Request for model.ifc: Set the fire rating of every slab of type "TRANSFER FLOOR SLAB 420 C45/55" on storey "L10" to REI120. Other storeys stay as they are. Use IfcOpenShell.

First a look at what the model holds.

```python
import ifcopenshell
import ifcopenshell.util.element

model = ifcopenshell.open("model.ifc")
print(model.schema)
storey = next(s for s in model.by_type("IfcBuildingStorey") if s.Name == "L10")
slabs = [e for e in ifcopenshell.util.element.get_decomposition(storey) if e.is_a("IfcSlab")]
seen = {}
for e in slabs:
    element_type = ifcopenshell.util.element.get_type(e)
    key = (element_type.Name if element_type != e and element_type else None, ifcopenshell.util.element.get_pset(e, "Pset_SlabCommon", "FireRating"))
    seen[key] = seen.get(key, 0) + 1
for (name, value), count in sorted(seen.items(), key=str):
    print(count, "x", name, "|", value)
```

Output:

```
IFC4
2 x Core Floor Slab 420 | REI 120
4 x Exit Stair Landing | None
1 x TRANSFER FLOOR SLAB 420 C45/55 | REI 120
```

```python
import ifcopenshell
import ifcopenshell.api.pset
import ifcopenshell.util.element

model = ifcopenshell.open("model.ifc")

storey = next(s for s in model.by_type("IfcBuildingStorey") if s.Name == "L10")
slabs = [e for e in ifcopenshell.util.element.get_decomposition(storey) if e.is_a("IfcSlab")]

count = 0
for e in slabs:
    element_type = ifcopenshell.util.element.get_type(e)
    if element_type in (None, e) or element_type.Name != "TRANSFER FLOOR SLAB 420 C45/55":
        continue
    found = ifcopenshell.util.element.get_pset(e, "Pset_SlabCommon", should_inherit=False)
    if found:
        pset = model.by_id(found["id"])
        if len(ifcopenshell.util.element.get_elements_by_pset(pset)) > 1:
            pset = ifcopenshell.api.pset.unshare_pset(model, products=[e], pset=pset)[0]
    else:
        pset = ifcopenshell.api.pset.add_pset(model, product=e, name="Pset_SlabCommon")
    ifcopenshell.api.pset.edit_pset(model, pset=pset, properties={"FireRating": "REI120"})
    count += 1

print(count, "slabs updated")

model.write("model_rev.ifc")
```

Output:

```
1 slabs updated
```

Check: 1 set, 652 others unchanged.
